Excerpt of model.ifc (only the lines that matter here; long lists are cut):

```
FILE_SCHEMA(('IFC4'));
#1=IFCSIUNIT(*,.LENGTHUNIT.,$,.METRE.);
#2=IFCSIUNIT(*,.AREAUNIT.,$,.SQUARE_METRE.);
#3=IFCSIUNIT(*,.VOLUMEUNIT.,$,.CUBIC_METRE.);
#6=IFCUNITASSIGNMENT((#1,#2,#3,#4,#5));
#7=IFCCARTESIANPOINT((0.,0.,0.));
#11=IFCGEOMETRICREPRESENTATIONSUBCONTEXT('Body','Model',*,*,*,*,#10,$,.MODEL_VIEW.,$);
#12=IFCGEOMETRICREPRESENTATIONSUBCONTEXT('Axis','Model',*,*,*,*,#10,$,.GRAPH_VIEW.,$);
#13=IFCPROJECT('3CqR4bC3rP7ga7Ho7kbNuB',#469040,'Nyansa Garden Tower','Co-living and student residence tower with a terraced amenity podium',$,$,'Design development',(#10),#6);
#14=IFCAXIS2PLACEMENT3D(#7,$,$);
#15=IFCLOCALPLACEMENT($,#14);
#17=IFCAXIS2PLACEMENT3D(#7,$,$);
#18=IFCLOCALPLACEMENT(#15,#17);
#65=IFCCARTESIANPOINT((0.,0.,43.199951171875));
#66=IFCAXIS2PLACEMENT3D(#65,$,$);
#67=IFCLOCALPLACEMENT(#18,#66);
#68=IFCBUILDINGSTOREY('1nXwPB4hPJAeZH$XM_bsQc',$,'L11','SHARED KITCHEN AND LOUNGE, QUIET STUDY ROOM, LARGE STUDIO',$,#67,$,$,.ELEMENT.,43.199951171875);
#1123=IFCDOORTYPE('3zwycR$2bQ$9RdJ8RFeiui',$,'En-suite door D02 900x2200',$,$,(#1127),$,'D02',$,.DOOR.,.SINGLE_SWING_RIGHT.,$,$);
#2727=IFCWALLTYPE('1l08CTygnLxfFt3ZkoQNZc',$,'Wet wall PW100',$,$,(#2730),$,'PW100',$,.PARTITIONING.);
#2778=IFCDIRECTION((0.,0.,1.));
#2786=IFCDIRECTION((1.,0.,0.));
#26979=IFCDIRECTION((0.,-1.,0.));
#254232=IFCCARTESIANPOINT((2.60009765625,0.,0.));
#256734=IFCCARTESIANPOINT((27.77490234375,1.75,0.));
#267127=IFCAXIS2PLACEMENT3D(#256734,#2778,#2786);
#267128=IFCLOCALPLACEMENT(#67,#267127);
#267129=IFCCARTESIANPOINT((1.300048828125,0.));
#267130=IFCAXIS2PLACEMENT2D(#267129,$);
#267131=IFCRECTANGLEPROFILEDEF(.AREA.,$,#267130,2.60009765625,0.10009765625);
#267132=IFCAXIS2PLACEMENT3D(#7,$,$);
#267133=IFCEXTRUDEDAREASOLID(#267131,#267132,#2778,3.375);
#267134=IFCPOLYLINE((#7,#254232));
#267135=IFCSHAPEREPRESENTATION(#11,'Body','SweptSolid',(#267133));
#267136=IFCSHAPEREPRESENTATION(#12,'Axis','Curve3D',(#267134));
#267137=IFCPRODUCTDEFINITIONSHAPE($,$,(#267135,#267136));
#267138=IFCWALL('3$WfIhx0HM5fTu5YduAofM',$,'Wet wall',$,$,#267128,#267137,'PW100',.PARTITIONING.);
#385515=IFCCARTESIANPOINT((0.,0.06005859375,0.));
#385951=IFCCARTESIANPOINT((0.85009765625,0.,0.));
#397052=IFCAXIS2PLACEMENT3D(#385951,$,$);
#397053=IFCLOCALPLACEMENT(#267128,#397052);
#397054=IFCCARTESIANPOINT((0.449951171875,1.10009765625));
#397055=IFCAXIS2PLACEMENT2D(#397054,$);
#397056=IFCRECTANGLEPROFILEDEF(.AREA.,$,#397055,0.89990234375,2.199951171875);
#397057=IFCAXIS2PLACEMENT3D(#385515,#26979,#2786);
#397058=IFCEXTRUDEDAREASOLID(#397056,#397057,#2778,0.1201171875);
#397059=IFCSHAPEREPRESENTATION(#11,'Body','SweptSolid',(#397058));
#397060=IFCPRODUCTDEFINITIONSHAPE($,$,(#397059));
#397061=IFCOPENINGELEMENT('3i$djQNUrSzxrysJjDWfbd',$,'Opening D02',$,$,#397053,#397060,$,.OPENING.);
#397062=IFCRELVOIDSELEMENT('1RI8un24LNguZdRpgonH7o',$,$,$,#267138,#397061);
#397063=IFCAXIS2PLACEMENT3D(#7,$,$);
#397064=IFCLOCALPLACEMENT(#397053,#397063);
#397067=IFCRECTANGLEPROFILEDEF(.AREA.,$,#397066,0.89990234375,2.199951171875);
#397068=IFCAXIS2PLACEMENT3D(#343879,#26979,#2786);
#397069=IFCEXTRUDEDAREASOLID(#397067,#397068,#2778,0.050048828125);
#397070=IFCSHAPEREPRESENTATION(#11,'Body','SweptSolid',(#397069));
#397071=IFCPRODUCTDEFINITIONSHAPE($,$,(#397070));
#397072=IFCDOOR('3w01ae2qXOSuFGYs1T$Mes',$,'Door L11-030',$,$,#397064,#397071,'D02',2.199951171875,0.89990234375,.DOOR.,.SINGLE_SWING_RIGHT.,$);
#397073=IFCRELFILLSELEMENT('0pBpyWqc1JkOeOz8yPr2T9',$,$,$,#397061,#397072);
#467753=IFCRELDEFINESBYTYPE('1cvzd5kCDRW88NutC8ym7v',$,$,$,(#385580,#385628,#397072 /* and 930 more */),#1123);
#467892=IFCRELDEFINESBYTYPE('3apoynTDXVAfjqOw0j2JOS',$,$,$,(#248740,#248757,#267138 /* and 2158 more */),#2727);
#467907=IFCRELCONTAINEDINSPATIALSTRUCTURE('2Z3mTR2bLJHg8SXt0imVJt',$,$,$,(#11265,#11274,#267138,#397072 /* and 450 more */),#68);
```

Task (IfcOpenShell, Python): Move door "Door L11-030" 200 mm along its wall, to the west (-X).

```python
import ifcopenshell
import ifcopenshell.api.geometry
import ifcopenshell.util.placement
import ifcopenshell.util.unit

model = ifcopenshell.open("model.ifc")
unit_scale = ifcopenshell.util.unit.calculate_unit_scale(model)

door = model.by_guid("3w01ae2qXOSuFGYs1T$Mes")
opening = door.FillsVoids[0].RelatingOpeningElement
wall = opening.VoidsElements[0].RelatingBuildingElement

wall_matrix = ifcopenshell.util.placement.get_local_placement(wall.ObjectPlacement)
shift = wall_matrix[:3, 0] * -0.2 / unit_scale
before = ifcopenshell.util.placement.get_local_placement(door.ObjectPlacement)[:3, 3].copy()

# The door is placed relative to its opening, so it follows when the opening moves.
matrix = ifcopenshell.util.placement.get_local_placement(opening.ObjectPlacement)
matrix[:3, 3] += shift
ifcopenshell.api.geometry.edit_object_placement(
    model, product=opening, matrix=matrix, is_si=False, should_transform_children=True
)

after = ifcopenshell.util.placement.get_local_placement(door.ObjectPlacement)[:3, 3]
print("door moved by", (after - before).round(3) + 0.0)

model.write("model_v2.ifc")
```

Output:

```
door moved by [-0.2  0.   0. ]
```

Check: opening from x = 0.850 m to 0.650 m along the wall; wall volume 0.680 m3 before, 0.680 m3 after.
